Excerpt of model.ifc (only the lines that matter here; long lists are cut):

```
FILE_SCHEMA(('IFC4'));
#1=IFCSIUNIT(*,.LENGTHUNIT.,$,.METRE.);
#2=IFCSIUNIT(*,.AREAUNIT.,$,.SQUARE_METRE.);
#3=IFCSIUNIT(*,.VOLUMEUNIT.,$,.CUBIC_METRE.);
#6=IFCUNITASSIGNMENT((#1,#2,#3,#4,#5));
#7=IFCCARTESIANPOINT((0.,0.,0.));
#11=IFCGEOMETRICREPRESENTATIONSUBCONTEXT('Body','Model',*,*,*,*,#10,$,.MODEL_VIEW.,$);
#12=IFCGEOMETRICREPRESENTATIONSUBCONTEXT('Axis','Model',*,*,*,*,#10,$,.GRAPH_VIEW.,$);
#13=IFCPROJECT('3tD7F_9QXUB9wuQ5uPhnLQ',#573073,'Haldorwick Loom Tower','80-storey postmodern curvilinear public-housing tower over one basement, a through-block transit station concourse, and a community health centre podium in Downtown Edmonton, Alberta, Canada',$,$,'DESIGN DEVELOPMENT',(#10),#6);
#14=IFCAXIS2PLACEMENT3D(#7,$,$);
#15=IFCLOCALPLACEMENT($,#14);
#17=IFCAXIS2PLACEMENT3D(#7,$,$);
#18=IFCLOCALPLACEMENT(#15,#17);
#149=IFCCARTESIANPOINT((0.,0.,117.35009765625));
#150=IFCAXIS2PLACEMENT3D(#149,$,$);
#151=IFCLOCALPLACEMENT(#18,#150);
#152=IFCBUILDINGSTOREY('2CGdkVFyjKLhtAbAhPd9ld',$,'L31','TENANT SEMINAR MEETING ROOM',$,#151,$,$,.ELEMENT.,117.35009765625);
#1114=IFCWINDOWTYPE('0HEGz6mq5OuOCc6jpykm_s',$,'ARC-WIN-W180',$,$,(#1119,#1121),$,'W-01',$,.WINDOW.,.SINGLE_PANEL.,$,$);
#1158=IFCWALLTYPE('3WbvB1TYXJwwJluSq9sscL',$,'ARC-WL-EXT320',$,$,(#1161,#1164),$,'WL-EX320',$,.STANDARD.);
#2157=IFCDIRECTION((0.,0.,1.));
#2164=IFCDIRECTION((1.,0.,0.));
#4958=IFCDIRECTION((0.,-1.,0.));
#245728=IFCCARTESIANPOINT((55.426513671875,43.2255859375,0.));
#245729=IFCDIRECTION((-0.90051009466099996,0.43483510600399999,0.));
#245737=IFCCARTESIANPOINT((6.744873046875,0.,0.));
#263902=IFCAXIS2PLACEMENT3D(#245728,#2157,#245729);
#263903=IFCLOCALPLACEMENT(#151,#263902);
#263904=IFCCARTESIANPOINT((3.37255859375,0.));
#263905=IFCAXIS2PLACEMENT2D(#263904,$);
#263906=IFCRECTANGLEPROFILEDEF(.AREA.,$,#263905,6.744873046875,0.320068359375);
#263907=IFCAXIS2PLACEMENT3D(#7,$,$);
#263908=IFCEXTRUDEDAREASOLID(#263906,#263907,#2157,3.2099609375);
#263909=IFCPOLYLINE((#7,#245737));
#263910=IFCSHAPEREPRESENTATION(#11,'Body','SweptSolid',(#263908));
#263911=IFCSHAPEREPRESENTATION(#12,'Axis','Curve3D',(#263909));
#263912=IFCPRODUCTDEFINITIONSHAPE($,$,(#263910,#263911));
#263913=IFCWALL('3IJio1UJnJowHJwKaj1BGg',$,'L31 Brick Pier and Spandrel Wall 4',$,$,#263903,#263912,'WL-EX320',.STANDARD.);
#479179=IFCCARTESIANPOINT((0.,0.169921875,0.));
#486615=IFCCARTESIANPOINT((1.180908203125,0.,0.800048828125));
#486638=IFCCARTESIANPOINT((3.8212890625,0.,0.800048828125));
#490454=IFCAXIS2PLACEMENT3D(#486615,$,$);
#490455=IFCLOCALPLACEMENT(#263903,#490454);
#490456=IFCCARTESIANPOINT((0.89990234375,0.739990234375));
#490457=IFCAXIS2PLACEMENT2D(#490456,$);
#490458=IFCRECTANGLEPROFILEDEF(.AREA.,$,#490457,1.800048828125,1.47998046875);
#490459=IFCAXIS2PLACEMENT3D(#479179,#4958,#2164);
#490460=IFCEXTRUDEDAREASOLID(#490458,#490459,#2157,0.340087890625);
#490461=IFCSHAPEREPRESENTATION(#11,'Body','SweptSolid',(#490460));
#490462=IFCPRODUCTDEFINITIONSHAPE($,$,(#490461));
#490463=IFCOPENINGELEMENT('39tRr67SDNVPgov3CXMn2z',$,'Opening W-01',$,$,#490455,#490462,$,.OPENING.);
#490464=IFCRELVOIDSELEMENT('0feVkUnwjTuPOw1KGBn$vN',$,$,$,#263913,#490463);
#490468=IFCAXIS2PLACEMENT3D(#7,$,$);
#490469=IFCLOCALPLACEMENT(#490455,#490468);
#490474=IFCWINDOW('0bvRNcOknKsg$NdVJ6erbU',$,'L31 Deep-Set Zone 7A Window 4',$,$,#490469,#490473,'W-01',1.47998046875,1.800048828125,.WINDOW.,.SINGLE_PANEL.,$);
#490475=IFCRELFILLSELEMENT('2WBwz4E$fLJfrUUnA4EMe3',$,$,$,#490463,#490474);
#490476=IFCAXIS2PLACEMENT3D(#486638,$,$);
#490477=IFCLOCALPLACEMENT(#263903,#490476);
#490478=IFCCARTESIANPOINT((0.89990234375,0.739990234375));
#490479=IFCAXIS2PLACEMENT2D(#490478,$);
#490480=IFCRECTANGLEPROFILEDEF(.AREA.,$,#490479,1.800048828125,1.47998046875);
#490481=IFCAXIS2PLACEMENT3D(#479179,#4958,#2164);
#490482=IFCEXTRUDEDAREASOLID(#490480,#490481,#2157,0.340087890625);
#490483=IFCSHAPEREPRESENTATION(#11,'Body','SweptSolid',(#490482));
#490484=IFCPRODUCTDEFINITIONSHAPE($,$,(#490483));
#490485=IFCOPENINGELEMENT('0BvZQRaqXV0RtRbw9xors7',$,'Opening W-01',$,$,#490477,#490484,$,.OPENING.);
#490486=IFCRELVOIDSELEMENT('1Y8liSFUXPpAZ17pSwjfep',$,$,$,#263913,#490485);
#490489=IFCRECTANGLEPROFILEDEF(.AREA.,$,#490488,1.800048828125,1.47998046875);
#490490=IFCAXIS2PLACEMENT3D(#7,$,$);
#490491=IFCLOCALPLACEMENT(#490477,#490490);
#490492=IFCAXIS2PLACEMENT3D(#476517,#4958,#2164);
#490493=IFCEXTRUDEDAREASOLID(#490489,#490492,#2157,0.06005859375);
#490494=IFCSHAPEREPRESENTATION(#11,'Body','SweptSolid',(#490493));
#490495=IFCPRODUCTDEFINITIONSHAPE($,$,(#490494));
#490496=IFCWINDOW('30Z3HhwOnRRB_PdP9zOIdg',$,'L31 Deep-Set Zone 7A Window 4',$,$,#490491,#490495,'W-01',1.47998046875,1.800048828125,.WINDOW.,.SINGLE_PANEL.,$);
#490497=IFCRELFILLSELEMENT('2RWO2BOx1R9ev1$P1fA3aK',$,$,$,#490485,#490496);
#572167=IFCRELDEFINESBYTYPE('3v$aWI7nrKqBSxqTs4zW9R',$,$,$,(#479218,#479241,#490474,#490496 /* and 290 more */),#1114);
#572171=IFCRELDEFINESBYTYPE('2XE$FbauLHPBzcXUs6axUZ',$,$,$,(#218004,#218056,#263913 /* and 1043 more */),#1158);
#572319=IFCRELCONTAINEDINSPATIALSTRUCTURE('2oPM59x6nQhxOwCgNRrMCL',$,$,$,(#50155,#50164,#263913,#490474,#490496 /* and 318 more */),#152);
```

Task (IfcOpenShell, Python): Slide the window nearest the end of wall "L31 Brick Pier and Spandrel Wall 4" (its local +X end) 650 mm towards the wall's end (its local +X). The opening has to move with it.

```python
import ifcopenshell
import ifcopenshell.api.geometry
import ifcopenshell.util.placement
import ifcopenshell.util.unit

model = ifcopenshell.open("model.ifc")
unit_scale = ifcopenshell.util.unit.calculate_unit_scale(model)

window = model.by_guid("30Z3HhwOnRRB_PdP9zOIdg")
opening = window.FillsVoids[0].RelatingOpeningElement
wall = opening.VoidsElements[0].RelatingBuildingElement

wall_matrix = ifcopenshell.util.placement.get_local_placement(wall.ObjectPlacement)
shift = wall_matrix[:3, 0] * 0.65 / unit_scale
before = ifcopenshell.util.placement.get_local_placement(window.ObjectPlacement)[:3, 3].copy()

# The window is placed relative to its opening, so it follows when the opening moves.
matrix = ifcopenshell.util.placement.get_local_placement(opening.ObjectPlacement)
matrix[:3, 3] += shift
ifcopenshell.api.geometry.edit_object_placement(
    model, product=opening, matrix=matrix, is_si=False, should_transform_children=True
)

after = ifcopenshell.util.placement.get_local_placement(window.ObjectPlacement)[:3, 3]
print("window moved by", (after - before).round(3) + 0.0)

model.write("model_rev.ifc")
```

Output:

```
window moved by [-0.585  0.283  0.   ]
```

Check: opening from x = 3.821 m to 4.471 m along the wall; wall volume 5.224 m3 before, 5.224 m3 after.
